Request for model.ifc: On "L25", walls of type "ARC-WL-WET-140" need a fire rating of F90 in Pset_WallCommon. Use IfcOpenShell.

First a look at what the model holds.

```python
import ifcopenshell
import ifcopenshell.util.element

model = ifcopenshell.open("model.ifc")
print(model.schema)
storey = next(s for s in model.by_type("IfcBuildingStorey") if s.Name == "L25")
walls = [e for e in ifcopenshell.util.element.get_decomposition(storey) if e.is_a("IfcWall")]
seen = {}
for e in walls:
    element_type = ifcopenshell.util.element.get_type(e)
    key = (element_type.Name if element_type != e and element_type else None, ifcopenshell.util.element.get_pset(e, "Pset_WallCommon", "FireRating"))
    seen[key] = seen.get(key, 0) + 1
for (name, value), count in sorted(seen.items(), key=str):
    print(count, "x", name, "|", value)
```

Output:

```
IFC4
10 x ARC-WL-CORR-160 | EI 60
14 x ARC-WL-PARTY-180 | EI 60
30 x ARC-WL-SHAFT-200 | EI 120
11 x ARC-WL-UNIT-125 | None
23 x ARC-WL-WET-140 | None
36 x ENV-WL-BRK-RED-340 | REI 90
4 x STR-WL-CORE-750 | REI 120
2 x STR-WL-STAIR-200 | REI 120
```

```python
import ifcopenshell
import ifcopenshell.api.pset
import ifcopenshell.util.element

model = ifcopenshell.open("model.ifc")

storey = next(s for s in model.by_type("IfcBuildingStorey") if s.Name == "L25")
walls = [e for e in ifcopenshell.util.element.get_decomposition(storey) if e.is_a("IfcWall")]

count = 0
for e in walls:
    element_type = ifcopenshell.util.element.get_type(e)
    if element_type in (None, e) or element_type.Name != "ARC-WL-WET-140":
        continue
    # add_pset returns the element's existing set when there is one.
    pset = ifcopenshell.api.pset.add_pset(model, product=e, name="Pset_WallCommon")
    ifcopenshell.api.pset.edit_pset(model, pset=pset, properties={"FireRating": "F90"})
    count += 1

print(count, "walls updated")

model.write("model_v2.ifc")
```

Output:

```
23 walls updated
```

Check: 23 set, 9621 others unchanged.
